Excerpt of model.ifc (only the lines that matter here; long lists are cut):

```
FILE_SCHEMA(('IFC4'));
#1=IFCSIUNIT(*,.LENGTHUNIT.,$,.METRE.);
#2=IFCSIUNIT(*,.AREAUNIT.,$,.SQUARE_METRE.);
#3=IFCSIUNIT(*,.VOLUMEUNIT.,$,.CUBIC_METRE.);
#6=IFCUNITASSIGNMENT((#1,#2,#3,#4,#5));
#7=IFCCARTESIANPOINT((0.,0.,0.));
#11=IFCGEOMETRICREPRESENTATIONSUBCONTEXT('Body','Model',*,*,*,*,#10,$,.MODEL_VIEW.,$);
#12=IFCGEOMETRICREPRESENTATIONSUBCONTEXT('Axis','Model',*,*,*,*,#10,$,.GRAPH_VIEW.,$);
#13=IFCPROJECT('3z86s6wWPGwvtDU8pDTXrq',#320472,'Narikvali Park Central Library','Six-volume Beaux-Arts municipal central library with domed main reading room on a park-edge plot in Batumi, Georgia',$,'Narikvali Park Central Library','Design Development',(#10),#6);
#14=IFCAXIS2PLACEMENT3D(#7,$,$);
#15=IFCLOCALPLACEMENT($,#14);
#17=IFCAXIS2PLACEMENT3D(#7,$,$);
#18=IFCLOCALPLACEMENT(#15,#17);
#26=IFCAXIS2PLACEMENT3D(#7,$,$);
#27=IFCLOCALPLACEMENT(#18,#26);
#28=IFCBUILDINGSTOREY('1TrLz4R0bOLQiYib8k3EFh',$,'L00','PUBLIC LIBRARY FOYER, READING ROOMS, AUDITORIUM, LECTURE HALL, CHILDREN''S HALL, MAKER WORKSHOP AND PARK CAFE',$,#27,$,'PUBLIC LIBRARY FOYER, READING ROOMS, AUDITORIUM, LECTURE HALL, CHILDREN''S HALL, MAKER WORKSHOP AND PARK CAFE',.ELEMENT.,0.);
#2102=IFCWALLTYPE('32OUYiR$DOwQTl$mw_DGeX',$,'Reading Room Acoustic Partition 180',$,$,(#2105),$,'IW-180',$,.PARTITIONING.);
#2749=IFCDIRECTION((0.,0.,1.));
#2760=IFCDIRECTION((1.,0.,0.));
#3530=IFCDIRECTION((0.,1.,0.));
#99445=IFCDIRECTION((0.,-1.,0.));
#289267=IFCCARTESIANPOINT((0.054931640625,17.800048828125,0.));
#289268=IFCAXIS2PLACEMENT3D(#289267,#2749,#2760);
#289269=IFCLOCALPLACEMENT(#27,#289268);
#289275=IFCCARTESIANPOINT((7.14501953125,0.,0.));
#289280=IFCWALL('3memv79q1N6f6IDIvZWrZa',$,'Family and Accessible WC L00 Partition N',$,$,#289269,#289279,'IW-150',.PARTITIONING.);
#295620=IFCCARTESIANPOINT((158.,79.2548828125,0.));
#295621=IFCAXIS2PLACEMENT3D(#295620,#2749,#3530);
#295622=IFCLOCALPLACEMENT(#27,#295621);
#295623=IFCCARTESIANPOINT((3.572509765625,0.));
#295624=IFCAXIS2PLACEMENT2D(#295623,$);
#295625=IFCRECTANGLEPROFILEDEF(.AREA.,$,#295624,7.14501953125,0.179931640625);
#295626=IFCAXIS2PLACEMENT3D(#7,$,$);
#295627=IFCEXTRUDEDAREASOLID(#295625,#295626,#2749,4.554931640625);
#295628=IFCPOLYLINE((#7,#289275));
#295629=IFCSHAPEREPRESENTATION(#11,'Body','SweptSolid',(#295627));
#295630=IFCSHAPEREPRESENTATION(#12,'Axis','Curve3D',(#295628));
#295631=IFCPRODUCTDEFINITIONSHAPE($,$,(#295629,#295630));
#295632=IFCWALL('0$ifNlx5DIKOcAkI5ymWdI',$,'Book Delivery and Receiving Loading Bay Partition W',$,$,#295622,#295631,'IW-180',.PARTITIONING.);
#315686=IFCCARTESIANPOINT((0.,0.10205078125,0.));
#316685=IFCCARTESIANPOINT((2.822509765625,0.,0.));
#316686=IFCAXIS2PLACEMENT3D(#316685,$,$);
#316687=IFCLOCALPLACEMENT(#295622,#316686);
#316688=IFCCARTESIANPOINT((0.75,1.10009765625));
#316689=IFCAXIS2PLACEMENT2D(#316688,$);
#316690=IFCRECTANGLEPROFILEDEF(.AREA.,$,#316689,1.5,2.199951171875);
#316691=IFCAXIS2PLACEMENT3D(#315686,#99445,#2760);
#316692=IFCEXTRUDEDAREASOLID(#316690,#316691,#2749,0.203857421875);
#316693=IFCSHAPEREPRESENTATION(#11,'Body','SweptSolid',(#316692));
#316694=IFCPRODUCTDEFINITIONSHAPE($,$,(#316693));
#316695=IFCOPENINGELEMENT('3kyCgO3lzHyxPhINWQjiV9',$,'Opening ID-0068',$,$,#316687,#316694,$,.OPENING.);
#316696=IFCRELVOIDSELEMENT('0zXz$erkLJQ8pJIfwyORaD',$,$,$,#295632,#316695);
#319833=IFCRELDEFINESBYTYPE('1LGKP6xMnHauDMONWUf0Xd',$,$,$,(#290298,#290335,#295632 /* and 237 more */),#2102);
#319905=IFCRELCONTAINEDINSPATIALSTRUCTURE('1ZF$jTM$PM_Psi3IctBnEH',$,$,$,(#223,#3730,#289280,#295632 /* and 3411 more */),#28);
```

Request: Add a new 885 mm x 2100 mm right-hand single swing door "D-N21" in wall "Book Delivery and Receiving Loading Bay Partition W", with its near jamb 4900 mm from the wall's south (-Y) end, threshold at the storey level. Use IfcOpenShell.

```python
import numpy as np
import ifcopenshell
import ifcopenshell.api.feature
import ifcopenshell.api.geometry
import ifcopenshell.api.root
import ifcopenshell.api.spatial
import ifcopenshell.geom
import ifcopenshell.util.element
import ifcopenshell.util.placement
import ifcopenshell.util.representation
import ifcopenshell.util.shape
import ifcopenshell.util.unit

model = ifcopenshell.open("model.ifc")
unit_scale = ifcopenshell.util.unit.calculate_unit_scale(model)
settings = ifcopenshell.geom.settings()


def volume(element):
    """Net volume in cubic metres, openings subtracted."""
    shape = ifcopenshell.geom.create_shape(settings, element)
    return ifcopenshell.util.shape.get_volume(shape.geometry)


wall = model.by_guid("0$ifNlx5DIKOcAkI5ymWdI")
storey = ifcopenshell.util.element.get_container(wall, ifc_class="IfcBuildingStorey")
context = ifcopenshell.util.representation.get_context(model, "Model", "Body", "MODEL_VIEW")
before = volume(wall)

width, height, from_end, sill = 0.885, 2.1, 4.9, 0.0  # metres

# The wall runs along its own X axis, and the end named is its -X end.
wall_shape = ifcopenshell.geom.create_shape(settings, wall)
x, y, z = ifcopenshell.util.shape.get_vertices(wall_shape.geometry).T
start = x.min() + from_end
face, thickness = float(y.min()), float(y.max() - y.min())
wall_matrix = ifcopenshell.util.placement.get_local_placement(wall.ObjectPlacement)
level = ifcopenshell.util.placement.get_local_placement(storey.ObjectPlacement)[2, 3]


def in_wall(x, y):
    """Placement at x, y metres in the wall's axes, at sill height."""
    matrix = wall_matrix.copy()
    matrix[:, 3] = wall_matrix @ np.array([x / unit_scale, y / unit_scale, 0.0, 1.0])
    matrix[2, 3] = level + sill / unit_scale
    return matrix


# Opening: a box that overshoots both wall faces by 50 mm.
opening = ifcopenshell.api.root.create_entity(model, ifc_class="IfcOpeningElement", predefined_type="OPENING")
box = ifcopenshell.api.geometry.add_wall_representation(
    model, context=context, length=width, height=height, thickness=thickness + 0.1
)
ifcopenshell.api.geometry.assign_representation(model, product=opening, representation=box)
ifcopenshell.api.geometry.edit_object_placement(model, product=opening, matrix=in_wall(start, face - 0.05), is_si=False)
ifcopenshell.api.feature.add_feature(model, feature=opening, element=wall)

door = ifcopenshell.api.root.create_entity(model, ifc_class="IfcDoor", name="D-N21", predefined_type="DOOR")
door.OverallWidth, door.OverallHeight = width / unit_scale, height / unit_scale
door.OperationType = "SINGLE_SWING_RIGHT"
body = ifcopenshell.api.geometry.add_door_representation(
    model,
    context=context,
    overall_width=door.OverallWidth,
    overall_height=door.OverallHeight,
    operation_type="SINGLE_SWING_RIGHT",
    lining_properties={"LiningDepth": thickness / unit_scale, "ThresholdDepth": thickness / unit_scale},
)
ifcopenshell.api.geometry.assign_representation(model, product=door, representation=body)
ifcopenshell.api.spatial.assign_container(model, products=[door], relating_structure=storey)
ifcopenshell.api.feature.add_filling(model, opening=opening, element=door)

# The lining spans the wall, so the door starts at the wall face.
ifcopenshell.api.geometry.edit_object_placement(model, product=door, matrix=in_wall(start, face), is_si=False)

after = volume(wall)

print(f"wall volume {before:.3f} -> {after:.3f} m3")

model.write("model-out.ifc")
```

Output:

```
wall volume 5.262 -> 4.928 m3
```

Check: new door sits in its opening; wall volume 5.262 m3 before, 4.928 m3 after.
